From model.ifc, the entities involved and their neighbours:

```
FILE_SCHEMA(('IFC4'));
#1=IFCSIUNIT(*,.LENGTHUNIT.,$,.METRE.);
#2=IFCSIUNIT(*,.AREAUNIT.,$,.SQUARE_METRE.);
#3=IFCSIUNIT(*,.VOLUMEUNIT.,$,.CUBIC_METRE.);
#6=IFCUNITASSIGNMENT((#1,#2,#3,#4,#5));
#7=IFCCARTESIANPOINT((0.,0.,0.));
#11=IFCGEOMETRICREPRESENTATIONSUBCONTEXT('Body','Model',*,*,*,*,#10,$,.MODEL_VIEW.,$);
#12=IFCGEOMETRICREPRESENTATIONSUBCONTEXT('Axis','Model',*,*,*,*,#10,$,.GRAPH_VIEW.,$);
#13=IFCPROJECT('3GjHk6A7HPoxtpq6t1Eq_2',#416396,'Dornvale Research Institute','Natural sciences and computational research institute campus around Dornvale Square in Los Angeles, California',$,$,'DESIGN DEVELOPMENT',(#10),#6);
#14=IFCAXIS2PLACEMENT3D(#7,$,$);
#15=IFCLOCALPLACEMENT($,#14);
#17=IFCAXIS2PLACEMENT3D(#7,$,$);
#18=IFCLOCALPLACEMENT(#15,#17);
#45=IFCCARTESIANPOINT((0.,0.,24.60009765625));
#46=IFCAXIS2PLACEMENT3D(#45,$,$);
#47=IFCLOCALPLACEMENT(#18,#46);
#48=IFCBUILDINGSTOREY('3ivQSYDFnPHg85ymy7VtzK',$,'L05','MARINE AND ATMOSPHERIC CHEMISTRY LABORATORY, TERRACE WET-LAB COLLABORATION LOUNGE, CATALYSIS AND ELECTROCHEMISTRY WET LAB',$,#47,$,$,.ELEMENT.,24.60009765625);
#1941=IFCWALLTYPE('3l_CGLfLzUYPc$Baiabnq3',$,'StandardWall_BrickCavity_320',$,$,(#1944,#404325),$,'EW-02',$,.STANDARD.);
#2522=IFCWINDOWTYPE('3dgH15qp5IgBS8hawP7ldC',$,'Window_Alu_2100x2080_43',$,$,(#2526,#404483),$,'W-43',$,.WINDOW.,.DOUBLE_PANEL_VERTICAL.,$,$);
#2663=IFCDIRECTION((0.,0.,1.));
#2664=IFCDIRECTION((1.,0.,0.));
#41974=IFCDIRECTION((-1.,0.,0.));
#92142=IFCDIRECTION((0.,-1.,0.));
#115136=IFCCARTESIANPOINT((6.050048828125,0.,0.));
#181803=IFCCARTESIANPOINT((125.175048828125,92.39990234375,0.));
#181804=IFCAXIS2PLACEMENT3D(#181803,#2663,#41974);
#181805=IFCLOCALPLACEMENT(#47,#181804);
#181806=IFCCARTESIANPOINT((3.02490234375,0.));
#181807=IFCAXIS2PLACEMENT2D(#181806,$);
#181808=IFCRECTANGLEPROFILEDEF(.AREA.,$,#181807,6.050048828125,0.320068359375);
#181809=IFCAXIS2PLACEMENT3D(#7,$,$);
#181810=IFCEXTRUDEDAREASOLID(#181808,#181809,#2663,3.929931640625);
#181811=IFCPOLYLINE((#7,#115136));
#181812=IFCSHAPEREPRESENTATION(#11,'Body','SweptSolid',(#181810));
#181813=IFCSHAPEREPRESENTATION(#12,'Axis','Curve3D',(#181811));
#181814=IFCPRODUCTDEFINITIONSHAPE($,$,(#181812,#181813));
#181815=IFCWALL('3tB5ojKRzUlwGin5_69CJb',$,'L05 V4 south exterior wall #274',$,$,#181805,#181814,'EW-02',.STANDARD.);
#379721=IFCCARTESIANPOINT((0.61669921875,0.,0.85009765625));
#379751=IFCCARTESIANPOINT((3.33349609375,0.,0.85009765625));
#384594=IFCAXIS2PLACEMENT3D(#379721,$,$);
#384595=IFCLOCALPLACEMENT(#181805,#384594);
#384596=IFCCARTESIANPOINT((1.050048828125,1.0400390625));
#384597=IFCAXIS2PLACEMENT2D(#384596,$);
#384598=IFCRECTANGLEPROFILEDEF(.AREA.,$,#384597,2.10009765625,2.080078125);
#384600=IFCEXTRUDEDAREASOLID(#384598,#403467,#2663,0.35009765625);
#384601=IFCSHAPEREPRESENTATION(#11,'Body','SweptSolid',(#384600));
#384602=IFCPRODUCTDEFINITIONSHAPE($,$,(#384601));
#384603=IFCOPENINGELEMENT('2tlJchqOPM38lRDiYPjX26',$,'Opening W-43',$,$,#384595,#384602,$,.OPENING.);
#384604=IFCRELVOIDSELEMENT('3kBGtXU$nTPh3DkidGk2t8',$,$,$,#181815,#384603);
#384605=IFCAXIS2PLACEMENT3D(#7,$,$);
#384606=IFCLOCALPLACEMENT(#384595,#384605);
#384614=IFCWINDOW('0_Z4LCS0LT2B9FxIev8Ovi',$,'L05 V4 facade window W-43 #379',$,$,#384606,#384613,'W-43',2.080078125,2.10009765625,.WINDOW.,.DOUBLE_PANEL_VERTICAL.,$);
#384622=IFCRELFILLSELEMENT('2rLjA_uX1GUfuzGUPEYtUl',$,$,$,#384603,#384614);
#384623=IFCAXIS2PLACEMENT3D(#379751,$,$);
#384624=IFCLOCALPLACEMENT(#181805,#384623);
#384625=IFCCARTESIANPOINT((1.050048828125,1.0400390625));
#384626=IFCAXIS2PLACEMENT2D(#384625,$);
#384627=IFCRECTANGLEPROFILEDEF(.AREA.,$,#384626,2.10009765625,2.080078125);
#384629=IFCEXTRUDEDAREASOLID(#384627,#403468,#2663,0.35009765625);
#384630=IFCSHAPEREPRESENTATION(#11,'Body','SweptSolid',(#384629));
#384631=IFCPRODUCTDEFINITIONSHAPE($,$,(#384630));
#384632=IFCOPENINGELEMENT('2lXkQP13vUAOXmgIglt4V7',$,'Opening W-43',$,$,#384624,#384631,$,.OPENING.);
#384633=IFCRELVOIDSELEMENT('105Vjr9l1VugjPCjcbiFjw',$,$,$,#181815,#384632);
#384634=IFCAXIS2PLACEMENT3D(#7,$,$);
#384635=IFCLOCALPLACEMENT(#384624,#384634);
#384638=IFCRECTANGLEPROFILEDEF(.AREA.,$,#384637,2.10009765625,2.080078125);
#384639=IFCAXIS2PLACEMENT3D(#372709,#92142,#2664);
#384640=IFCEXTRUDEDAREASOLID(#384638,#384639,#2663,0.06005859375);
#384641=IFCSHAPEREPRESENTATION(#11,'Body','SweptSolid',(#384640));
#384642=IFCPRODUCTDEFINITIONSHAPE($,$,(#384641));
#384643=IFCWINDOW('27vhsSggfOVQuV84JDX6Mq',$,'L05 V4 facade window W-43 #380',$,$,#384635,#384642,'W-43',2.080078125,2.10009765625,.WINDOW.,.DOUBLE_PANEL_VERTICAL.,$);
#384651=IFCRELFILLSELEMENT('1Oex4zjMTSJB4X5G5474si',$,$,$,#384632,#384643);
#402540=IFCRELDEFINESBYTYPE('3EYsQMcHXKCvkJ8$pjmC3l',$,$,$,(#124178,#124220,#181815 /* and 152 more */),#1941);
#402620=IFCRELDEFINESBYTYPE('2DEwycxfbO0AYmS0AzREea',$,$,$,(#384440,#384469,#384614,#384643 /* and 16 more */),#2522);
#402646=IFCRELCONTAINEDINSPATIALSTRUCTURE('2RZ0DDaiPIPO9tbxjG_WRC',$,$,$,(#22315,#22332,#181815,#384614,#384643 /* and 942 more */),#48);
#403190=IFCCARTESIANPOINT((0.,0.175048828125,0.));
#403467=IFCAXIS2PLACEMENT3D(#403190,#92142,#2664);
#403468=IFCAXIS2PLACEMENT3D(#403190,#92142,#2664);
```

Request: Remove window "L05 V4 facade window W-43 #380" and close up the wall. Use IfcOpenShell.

```python
import ifcopenshell
import ifcopenshell.api.feature
import ifcopenshell.api.root
import ifcopenshell.geom
import ifcopenshell.util.shape

model = ifcopenshell.open("model.ifc")
settings = ifcopenshell.geom.settings()


def volume(element):
    """Net volume in cubic metres, openings subtracted."""
    shape = ifcopenshell.geom.create_shape(settings, element)
    return ifcopenshell.util.shape.get_volume(shape.geometry)


window = model.by_guid("27vhsSggfOVQuV84JDX6Mq")
opening = window.FillsVoids[0].RelatingOpeningElement
wall = opening.VoidsElements[0].RelatingBuildingElement
before = volume(wall)

ifcopenshell.api.root.remove_product(model, product=window)
ifcopenshell.api.feature.remove_feature(model, feature=opening)

after = volume(wall)

print(f"wall volume {before:.3f} -> {after:.3f} m3")

model.write("model_updated.ifc")
```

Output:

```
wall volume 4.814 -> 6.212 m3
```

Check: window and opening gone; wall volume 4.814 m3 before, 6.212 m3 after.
